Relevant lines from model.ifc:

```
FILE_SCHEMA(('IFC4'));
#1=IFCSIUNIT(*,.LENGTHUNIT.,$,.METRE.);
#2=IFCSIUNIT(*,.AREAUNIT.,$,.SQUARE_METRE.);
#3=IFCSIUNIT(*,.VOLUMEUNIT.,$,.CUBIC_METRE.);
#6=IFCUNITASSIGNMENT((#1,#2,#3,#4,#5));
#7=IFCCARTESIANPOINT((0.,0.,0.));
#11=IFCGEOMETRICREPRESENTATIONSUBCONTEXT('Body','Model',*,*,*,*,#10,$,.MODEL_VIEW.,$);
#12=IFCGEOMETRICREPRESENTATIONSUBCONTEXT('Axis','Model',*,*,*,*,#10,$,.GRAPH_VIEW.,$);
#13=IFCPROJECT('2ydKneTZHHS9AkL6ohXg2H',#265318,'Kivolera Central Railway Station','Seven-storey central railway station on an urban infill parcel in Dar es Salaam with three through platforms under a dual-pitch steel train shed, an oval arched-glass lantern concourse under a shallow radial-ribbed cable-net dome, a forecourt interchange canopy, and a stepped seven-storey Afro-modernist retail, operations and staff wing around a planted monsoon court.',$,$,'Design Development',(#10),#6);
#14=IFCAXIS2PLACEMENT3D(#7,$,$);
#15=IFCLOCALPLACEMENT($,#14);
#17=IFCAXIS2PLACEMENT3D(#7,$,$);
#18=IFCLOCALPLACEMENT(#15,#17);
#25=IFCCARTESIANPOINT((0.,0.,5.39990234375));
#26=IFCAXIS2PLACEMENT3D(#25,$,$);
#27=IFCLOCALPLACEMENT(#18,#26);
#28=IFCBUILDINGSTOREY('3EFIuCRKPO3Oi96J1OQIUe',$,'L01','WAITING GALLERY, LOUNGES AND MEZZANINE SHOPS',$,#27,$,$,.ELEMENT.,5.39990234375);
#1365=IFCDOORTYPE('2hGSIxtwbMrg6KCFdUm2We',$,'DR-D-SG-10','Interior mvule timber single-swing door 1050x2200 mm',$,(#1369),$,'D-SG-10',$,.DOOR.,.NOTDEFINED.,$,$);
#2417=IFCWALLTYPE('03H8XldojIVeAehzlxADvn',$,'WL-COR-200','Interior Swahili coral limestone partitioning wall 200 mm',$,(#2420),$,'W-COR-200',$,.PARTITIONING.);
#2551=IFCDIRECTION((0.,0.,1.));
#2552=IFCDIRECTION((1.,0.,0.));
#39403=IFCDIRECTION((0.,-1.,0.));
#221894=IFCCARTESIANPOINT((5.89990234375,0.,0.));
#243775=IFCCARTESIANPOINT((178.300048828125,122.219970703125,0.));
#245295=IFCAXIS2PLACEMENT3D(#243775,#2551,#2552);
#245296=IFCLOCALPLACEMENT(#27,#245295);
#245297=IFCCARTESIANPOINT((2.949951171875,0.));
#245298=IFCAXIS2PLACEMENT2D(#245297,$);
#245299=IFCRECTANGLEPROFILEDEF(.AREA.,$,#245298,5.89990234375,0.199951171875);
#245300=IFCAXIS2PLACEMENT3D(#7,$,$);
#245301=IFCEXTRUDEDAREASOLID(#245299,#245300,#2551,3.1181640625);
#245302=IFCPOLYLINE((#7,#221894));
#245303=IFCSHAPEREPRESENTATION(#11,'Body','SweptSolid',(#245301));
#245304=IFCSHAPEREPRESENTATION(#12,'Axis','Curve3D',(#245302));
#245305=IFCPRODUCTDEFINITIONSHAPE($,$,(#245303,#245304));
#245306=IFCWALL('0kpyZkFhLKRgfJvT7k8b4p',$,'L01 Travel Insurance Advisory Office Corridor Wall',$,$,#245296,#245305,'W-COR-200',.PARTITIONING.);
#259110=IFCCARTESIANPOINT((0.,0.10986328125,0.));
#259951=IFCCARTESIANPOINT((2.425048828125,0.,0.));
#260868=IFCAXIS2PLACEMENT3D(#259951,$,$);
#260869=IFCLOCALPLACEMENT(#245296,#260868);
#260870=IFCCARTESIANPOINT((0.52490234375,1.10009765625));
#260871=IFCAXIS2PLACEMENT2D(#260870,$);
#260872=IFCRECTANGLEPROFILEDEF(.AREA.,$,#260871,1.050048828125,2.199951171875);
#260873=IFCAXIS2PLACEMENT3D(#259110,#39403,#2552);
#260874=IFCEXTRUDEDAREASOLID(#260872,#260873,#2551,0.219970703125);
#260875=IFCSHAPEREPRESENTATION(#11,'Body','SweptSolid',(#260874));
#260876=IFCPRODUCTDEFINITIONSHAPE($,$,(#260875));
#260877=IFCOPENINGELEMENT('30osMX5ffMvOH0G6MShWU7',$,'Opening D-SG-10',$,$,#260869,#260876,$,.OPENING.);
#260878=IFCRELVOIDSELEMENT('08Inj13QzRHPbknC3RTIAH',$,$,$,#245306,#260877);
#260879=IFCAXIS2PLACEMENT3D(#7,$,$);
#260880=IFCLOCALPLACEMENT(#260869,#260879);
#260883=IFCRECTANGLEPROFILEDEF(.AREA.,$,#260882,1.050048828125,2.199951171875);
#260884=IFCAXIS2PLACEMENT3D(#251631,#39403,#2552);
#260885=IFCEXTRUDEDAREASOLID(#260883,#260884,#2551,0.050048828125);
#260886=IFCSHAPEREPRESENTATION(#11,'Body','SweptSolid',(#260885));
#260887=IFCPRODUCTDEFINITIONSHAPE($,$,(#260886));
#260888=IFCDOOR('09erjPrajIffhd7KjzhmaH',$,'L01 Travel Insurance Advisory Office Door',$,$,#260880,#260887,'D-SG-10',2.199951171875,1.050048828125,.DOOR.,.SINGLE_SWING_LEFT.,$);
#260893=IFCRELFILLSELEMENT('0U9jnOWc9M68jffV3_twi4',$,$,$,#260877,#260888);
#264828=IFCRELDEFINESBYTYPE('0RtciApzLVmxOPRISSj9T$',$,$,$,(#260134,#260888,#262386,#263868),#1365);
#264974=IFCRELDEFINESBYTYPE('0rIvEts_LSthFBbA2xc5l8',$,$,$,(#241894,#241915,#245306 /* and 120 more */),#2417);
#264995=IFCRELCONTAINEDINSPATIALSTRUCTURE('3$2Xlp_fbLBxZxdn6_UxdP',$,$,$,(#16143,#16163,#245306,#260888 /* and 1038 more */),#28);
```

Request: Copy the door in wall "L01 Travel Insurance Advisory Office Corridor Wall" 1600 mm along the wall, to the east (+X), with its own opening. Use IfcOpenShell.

```python
import ifcopenshell
import ifcopenshell.api.feature
import ifcopenshell.api.geometry
import ifcopenshell.api.root
import ifcopenshell.geom
import ifcopenshell.util.element
import ifcopenshell.util.placement
import ifcopenshell.util.shape

model = ifcopenshell.open("model.ifc")
settings = ifcopenshell.geom.settings()


def volume(element):
    """Net volume in cubic metres, openings subtracted."""
    shape = ifcopenshell.geom.create_shape(settings, element)
    return ifcopenshell.util.shape.get_volume(shape.geometry)


door = model.by_id(260888)
opening = door.FillsVoids[0].RelatingOpeningElement
wall = opening.VoidsElements[0].RelatingBuildingElement
before = volume(wall)
shift = ifcopenshell.util.placement.get_local_placement(wall.ObjectPlacement)[:3, 0] * 1.6

# copy_class copies the void relationship, type, container and properties, but no geometry.
new_opening = ifcopenshell.api.root.copy_class(model, product=opening)
new_opening.Representation = ifcopenshell.util.element.copy_deep(
    model, opening.Representation, exclude=["IfcGeometricRepresentationContext", "IfcRepresentationMap"]
)
new_door = ifcopenshell.api.root.copy_class(model, product=door)
new_door.Representation = ifcopenshell.util.element.copy_deep(
    model, door.Representation, exclude=["IfcGeometricRepresentationContext", "IfcRepresentationMap"]
)
new_door.Tag = None
ifcopenshell.api.feature.add_filling(model, opening=new_opening, element=new_door)

for old, new in ((opening, new_opening), (door, new_door)):
    matrix = ifcopenshell.util.placement.get_local_placement(old.ObjectPlacement)
    matrix[:3, 3] += shift
    ifcopenshell.api.geometry.edit_object_placement(model, product=new, matrix=matrix, is_si=False)

after = volume(wall)

print(f"wall volume {before:.3f} -> {after:.3f} m3")

model.write("model-out.ifc")
```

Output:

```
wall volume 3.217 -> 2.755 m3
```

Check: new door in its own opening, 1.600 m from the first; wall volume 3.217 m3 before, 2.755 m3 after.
